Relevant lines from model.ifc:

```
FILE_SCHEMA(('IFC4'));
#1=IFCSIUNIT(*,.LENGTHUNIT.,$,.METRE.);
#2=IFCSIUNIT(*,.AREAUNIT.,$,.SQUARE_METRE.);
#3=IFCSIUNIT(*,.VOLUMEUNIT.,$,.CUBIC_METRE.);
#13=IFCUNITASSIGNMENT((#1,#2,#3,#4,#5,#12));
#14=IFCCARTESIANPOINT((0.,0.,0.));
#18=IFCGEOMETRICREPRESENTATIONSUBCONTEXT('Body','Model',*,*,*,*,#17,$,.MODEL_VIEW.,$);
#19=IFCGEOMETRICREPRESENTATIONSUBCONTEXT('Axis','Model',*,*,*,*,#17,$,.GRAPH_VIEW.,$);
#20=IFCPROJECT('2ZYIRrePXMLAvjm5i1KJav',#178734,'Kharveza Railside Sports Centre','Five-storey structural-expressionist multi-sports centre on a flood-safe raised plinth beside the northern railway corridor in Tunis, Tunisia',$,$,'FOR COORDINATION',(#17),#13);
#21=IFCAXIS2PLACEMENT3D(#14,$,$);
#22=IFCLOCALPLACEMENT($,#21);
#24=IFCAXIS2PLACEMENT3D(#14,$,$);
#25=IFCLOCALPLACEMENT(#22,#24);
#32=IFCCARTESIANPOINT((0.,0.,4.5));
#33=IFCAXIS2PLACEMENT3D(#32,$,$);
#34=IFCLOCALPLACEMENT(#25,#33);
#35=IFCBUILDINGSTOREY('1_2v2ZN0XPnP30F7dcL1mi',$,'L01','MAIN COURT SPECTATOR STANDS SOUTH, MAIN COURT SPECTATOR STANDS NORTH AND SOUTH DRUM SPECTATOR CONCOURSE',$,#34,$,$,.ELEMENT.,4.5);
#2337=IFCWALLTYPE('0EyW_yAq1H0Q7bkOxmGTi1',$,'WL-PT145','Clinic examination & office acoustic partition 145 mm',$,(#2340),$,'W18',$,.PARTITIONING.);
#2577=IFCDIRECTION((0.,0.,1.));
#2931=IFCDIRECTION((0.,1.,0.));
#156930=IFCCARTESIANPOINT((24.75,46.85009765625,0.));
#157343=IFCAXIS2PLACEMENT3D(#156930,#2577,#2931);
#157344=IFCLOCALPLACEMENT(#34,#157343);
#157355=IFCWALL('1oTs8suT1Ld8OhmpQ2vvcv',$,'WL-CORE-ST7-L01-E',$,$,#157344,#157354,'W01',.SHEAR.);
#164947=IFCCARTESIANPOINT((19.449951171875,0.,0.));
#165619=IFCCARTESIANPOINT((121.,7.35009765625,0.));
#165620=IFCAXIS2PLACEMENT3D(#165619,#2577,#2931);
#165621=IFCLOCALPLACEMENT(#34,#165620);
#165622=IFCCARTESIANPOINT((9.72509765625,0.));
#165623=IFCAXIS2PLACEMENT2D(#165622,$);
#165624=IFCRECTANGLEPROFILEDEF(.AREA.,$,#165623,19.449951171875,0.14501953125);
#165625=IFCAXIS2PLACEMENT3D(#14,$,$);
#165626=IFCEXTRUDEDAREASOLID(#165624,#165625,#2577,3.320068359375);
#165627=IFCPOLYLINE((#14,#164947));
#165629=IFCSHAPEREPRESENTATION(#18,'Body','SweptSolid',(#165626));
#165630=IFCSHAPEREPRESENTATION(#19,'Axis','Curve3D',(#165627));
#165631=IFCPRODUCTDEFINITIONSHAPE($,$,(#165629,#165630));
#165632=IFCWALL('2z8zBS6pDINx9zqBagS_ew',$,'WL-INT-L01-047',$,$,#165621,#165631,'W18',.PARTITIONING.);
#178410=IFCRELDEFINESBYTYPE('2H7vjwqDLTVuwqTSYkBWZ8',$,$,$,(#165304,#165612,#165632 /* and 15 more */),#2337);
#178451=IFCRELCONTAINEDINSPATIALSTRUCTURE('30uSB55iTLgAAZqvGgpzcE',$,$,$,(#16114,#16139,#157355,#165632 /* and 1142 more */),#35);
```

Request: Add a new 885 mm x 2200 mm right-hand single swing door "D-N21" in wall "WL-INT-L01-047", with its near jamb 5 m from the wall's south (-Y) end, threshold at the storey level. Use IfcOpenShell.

```python
import numpy as np
import ifcopenshell
import ifcopenshell.api.feature
import ifcopenshell.api.geometry
import ifcopenshell.api.root
import ifcopenshell.api.spatial
import ifcopenshell.geom
import ifcopenshell.util.element
import ifcopenshell.util.placement
import ifcopenshell.util.representation
import ifcopenshell.util.shape
import ifcopenshell.util.unit

model = ifcopenshell.open("model.ifc")
unit_scale = ifcopenshell.util.unit.calculate_unit_scale(model)
settings = ifcopenshell.geom.settings()


def volume(element):
    """Net volume in cubic metres, openings subtracted."""
    shape = ifcopenshell.geom.create_shape(settings, element)
    return ifcopenshell.util.shape.get_volume(shape.geometry)


wall = model.by_guid("2z8zBS6pDINx9zqBagS_ew")
storey = ifcopenshell.util.element.get_container(wall, ifc_class="IfcBuildingStorey")
context = ifcopenshell.util.representation.get_context(model, "Model", "Body", "MODEL_VIEW")
before = volume(wall)

width, height, from_end, sill = 0.885, 2.2, 5, 0.0  # metres

# The wall runs along its own X axis, and the end named is its -X end.
wall_shape = ifcopenshell.geom.create_shape(settings, wall)
x, y, z = ifcopenshell.util.shape.get_vertices(wall_shape.geometry).T
start = x.min() + from_end
face, thickness = float(y.min()), float(y.max() - y.min())
wall_matrix = ifcopenshell.util.placement.get_local_placement(wall.ObjectPlacement)
level = ifcopenshell.util.placement.get_local_placement(storey.ObjectPlacement)[2, 3]


def in_wall(x, y):
    """Placement at x, y metres in the wall's axes, at sill height."""
    matrix = wall_matrix.copy()
    matrix[:, 3] = wall_matrix @ np.array([x / unit_scale, y / unit_scale, 0.0, 1.0])
    matrix[2, 3] = level + sill / unit_scale
    return matrix


# Opening: a box that overshoots both wall faces by 50 mm.
opening = ifcopenshell.api.root.create_entity(model, ifc_class="IfcOpeningElement", predefined_type="OPENING")
box = ifcopenshell.api.geometry.add_wall_representation(
    model, context=context, length=width, height=height, thickness=thickness + 0.1
)
ifcopenshell.api.geometry.assign_representation(model, product=opening, representation=box)
ifcopenshell.api.geometry.edit_object_placement(model, product=opening, matrix=in_wall(start, face - 0.05), is_si=False)
ifcopenshell.api.feature.add_feature(model, feature=opening, element=wall)

door = ifcopenshell.api.root.create_entity(model, ifc_class="IfcDoor", name="D-N21", predefined_type="DOOR")
door.OverallWidth, door.OverallHeight = width / unit_scale, height / unit_scale
door.OperationType = "SINGLE_SWING_RIGHT"
body = ifcopenshell.api.geometry.add_door_representation(
    model,
    context=context,
    overall_width=door.OverallWidth,
    overall_height=door.OverallHeight,
    operation_type="SINGLE_SWING_RIGHT",
    lining_properties={"LiningDepth": thickness / unit_scale, "ThresholdDepth": thickness / unit_scale},
)
ifcopenshell.api.geometry.assign_representation(model, product=door, representation=body)
ifcopenshell.api.spatial.assign_container(model, products=[door], relating_structure=storey)
ifcopenshell.api.feature.add_filling(model, opening=opening, element=door)

# The lining spans the wall, so the door starts at the wall face.
ifcopenshell.api.geometry.edit_object_placement(model, product=door, matrix=in_wall(start, face), is_si=False)

after = volume(wall)

print(f"wall volume {before:.3f} -> {after:.3f} m3")

model.write("model_updated.ifc")
```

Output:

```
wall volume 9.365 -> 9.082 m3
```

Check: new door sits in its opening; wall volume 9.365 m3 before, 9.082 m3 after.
